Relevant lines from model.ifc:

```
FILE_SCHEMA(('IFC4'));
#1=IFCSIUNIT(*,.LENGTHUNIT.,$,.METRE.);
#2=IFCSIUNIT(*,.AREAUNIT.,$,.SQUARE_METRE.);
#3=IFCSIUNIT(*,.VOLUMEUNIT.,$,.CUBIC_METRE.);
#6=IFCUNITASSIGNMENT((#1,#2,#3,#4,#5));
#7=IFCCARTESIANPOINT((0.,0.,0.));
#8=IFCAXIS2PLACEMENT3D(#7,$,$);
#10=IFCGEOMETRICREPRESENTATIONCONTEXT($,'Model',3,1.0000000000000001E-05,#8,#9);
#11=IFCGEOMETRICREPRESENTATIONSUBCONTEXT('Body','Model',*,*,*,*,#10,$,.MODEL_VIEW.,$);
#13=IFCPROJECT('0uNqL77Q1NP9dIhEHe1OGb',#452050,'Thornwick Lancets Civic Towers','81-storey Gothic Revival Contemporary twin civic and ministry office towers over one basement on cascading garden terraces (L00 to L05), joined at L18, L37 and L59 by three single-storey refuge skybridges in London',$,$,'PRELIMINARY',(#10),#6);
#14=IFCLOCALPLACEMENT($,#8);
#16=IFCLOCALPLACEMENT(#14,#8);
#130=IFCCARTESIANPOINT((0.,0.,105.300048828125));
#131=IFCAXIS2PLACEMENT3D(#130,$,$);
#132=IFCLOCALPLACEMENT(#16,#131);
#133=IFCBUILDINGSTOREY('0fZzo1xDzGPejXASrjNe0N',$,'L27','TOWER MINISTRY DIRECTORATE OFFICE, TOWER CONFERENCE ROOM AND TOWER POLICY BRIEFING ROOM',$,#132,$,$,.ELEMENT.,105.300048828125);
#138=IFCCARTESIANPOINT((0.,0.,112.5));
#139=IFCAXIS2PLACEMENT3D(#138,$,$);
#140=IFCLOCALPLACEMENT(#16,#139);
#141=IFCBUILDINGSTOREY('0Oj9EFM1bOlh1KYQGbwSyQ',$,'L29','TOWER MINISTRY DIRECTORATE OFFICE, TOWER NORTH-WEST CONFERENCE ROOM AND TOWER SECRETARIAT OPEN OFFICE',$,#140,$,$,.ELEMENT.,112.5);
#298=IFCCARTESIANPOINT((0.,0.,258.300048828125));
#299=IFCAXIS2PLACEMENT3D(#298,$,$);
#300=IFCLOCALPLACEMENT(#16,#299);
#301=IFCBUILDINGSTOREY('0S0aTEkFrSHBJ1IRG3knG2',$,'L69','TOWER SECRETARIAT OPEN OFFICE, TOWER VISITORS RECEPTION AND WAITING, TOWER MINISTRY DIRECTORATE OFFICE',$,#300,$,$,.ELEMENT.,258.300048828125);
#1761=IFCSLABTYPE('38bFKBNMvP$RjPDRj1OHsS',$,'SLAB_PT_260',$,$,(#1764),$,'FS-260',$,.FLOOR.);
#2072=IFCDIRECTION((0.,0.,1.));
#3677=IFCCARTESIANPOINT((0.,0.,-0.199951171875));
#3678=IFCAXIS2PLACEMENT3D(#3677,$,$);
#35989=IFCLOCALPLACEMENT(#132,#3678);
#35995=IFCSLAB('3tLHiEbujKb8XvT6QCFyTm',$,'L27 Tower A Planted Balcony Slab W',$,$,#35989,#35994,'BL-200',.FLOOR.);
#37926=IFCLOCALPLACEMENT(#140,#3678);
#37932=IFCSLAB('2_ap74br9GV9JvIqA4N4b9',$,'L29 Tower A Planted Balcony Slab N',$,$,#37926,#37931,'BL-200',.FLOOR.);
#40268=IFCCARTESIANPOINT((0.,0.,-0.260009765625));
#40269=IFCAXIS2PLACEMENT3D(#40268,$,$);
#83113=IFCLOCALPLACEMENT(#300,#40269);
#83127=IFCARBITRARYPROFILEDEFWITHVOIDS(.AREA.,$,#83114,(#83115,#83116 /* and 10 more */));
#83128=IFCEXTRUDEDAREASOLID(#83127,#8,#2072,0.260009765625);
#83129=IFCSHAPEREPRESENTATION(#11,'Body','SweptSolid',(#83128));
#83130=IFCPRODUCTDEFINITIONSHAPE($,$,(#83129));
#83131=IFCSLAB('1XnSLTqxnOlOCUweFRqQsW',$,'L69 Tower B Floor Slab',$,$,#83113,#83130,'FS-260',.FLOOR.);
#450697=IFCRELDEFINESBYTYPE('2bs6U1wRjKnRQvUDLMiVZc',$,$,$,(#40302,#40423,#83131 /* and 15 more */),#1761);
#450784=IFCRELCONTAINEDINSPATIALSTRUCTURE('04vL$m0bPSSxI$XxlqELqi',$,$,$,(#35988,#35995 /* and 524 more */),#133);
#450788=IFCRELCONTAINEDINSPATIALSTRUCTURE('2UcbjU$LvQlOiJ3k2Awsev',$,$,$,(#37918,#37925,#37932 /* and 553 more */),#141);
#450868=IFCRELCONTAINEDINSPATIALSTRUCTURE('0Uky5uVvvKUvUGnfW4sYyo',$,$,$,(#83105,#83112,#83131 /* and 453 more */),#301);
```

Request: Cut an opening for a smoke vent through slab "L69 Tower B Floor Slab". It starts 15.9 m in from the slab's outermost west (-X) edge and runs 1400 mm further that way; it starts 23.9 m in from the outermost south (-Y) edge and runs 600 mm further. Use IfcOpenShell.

```python
import numpy as np
import ifcopenshell
import ifcopenshell.api.feature
import ifcopenshell.api.geometry
import ifcopenshell.api.root
import ifcopenshell.geom
import ifcopenshell.util.placement
import ifcopenshell.util.representation
import ifcopenshell.util.shape
import ifcopenshell.util.unit

model = ifcopenshell.open("model.ifc")
unit_scale = ifcopenshell.util.unit.calculate_unit_scale(model)
settings = ifcopenshell.geom.settings()


def volume(element):
    """Net volume in cubic metres, openings subtracted."""
    shape = ifcopenshell.geom.create_shape(settings, element)
    return ifcopenshell.util.shape.get_volume(shape.geometry)


slab = model.by_guid("1XnSLTqxnOlOCUweFRqQsW")
before = volume(slab)

# Extent in the slab's own axes, in metres. The edges named are its -X and -Y sides.
slab_shape = ifcopenshell.geom.create_shape(settings, slab)
vertices = ifcopenshell.util.shape.get_vertices(slab_shape.geometry)
x_min, y_min, bottom = vertices.min(axis=0)
top = vertices[:, 2].max()

opening = ifcopenshell.api.root.create_entity(model, ifc_class="IfcOpeningElement", name="Smoke vent opening", predefined_type="OPENING")
context = ifcopenshell.util.representation.get_context(model, "Model", "Body", "MODEL_VIEW")
width, depth = 1.4, 0.6
outline = [(0.0, 0.0), (width, 0.0), (width, depth), (0.0, depth), (0.0, 0.0)]
# Overshoot both faces by 50 mm so the cut is clean.
shape = ifcopenshell.api.geometry.add_slab_representation(
    model, context=context, depth=top - bottom + 0.1, polyline=outline
)
ifcopenshell.api.geometry.assign_representation(model, product=opening, representation=shape)

matrix = ifcopenshell.util.placement.get_local_placement(slab.ObjectPlacement)
matrix[:, 3] = matrix @ np.append(np.array([x_min + 15.9, y_min + 23.9, bottom - 0.05]) / unit_scale, 1.0)
ifcopenshell.api.geometry.edit_object_placement(model, product=opening, matrix=matrix, is_si=False)
ifcopenshell.api.feature.add_feature(model, feature=opening, element=slab)

after = volume(slab)

print(f"slab volume {before:.3f} -> {after:.3f} m3")

model.write("model-out.ifc")
```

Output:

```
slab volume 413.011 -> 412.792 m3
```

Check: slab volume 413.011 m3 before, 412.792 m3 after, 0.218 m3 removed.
